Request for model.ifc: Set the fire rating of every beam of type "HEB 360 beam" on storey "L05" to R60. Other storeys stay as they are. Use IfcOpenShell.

First a look at what the model holds.

```python
import ifcopenshell
import ifcopenshell.util.element

model = ifcopenshell.open("model.ifc")
print(model.schema)
storey = next(s for s in model.by_type("IfcBuildingStorey") if s.Name == "L05")
beams = [e for e in ifcopenshell.util.element.get_decomposition(storey) if e.is_a("IfcBeam")]
seen = {}
for e in beams:
    element_type = ifcopenshell.util.element.get_type(e)
    key = (element_type.Name if element_type != e and element_type else None, ifcopenshell.util.element.get_pset(e, "Pset_BeamCommon", "FireRating"))
    seen[key] = seen.get(key, 0) + 1
for (name, value), count in sorted(seen.items(), key=str):
    print(count, "x", name, "|", value)
```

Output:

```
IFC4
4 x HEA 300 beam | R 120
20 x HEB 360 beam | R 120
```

```python
import ifcopenshell
import ifcopenshell.api.pset
import ifcopenshell.util.element

model = ifcopenshell.open("model.ifc")

storey = next(s for s in model.by_type("IfcBuildingStorey") if s.Name == "L05")
beams = [e for e in ifcopenshell.util.element.get_decomposition(storey) if e.is_a("IfcBeam")]

count = 0
for e in beams:
    element_type = ifcopenshell.util.element.get_type(e)
    if element_type in (None, e) or element_type.Name != "HEB 360 beam":
        continue
    # add_pset returns the element's existing set when there is one.
    pset = ifcopenshell.api.pset.add_pset(model, product=e, name="Pset_BeamCommon")
    ifcopenshell.api.pset.edit_pset(model, pset=pset, properties={"FireRating": "R60"})
    count += 1

print(count, "beams updated")

model.write("model_updated.ifc")
```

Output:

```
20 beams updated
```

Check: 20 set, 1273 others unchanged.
